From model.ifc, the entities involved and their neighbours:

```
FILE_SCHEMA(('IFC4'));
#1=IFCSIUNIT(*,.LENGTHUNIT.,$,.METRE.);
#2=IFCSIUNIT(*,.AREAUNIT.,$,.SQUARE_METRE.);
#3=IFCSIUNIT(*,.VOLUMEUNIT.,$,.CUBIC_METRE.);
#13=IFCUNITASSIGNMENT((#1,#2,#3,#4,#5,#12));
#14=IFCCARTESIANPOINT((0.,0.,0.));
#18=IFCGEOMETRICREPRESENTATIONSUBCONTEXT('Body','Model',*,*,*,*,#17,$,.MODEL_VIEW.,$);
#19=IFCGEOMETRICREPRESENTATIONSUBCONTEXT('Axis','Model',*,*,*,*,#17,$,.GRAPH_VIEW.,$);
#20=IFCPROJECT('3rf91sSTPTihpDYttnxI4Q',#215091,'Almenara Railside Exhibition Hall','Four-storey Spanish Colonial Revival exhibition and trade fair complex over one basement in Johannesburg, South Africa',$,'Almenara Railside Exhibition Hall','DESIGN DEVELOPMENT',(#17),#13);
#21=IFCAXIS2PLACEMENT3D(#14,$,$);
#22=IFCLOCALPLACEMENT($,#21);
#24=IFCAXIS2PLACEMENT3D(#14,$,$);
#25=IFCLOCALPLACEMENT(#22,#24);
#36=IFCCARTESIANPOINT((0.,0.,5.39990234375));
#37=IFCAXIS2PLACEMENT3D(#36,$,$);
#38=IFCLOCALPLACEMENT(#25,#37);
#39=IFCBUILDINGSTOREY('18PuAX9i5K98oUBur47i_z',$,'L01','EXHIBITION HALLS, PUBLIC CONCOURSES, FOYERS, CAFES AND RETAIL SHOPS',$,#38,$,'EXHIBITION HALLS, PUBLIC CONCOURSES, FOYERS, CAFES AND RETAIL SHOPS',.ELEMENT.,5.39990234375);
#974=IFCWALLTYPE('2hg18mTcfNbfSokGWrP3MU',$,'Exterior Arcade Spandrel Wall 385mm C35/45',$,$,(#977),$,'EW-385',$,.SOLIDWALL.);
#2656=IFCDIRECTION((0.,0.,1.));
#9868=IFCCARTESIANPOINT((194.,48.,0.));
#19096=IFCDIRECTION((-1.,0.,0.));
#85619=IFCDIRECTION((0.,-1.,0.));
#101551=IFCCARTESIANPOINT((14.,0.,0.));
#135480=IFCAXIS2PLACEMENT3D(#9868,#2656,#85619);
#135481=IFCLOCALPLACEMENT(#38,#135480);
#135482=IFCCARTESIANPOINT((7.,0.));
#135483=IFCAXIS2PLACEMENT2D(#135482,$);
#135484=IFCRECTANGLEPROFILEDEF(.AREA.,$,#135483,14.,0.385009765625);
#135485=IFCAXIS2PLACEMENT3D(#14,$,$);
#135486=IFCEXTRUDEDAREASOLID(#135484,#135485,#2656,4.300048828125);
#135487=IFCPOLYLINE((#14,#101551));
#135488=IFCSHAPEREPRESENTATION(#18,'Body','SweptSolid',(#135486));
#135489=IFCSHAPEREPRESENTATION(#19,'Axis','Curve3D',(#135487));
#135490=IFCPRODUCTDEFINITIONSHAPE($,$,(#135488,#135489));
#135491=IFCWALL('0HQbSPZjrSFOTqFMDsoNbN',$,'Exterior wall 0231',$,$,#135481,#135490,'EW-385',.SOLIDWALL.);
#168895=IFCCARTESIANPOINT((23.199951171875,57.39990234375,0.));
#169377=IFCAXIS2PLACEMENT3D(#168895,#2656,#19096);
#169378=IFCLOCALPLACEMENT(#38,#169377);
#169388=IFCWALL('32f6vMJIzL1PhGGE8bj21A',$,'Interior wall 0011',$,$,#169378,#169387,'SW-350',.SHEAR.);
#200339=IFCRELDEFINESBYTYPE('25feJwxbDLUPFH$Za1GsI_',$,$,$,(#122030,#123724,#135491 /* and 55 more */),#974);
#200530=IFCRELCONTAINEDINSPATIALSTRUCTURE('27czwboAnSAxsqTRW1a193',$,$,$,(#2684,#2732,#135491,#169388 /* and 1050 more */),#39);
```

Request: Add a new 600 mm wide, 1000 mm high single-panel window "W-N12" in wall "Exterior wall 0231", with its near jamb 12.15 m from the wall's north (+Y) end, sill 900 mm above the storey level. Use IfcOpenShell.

```python
import numpy as np
import ifcopenshell
import ifcopenshell.api.feature
import ifcopenshell.api.geometry
import ifcopenshell.api.root
import ifcopenshell.api.spatial
import ifcopenshell.geom
import ifcopenshell.util.element
import ifcopenshell.util.placement
import ifcopenshell.util.representation
import ifcopenshell.util.shape
import ifcopenshell.util.unit

model = ifcopenshell.open("model.ifc")
unit_scale = ifcopenshell.util.unit.calculate_unit_scale(model)
settings = ifcopenshell.geom.settings()


def volume(element):
    """Net volume in cubic metres, openings subtracted."""
    shape = ifcopenshell.geom.create_shape(settings, element)
    return ifcopenshell.util.shape.get_volume(shape.geometry)


wall = model.by_guid("0HQbSPZjrSFOTqFMDsoNbN")
storey = ifcopenshell.util.element.get_container(wall, ifc_class="IfcBuildingStorey")
context = ifcopenshell.util.representation.get_context(model, "Model", "Body", "MODEL_VIEW")
before = volume(wall)

width, height, from_end, sill = 0.6, 1, 12.15, 0.9  # metres

# The wall runs along its own X axis, and the end named is its -X end.
wall_shape = ifcopenshell.geom.create_shape(settings, wall)
x, y, z = ifcopenshell.util.shape.get_vertices(wall_shape.geometry).T
start = x.min() + from_end
face, thickness = float(y.min()), float(y.max() - y.min())
wall_matrix = ifcopenshell.util.placement.get_local_placement(wall.ObjectPlacement)
level = ifcopenshell.util.placement.get_local_placement(storey.ObjectPlacement)[2, 3]


def in_wall(x, y):
    """Placement at x, y metres in the wall's axes, at sill height."""
    matrix = wall_matrix.copy()
    matrix[:, 3] = wall_matrix @ np.array([x / unit_scale, y / unit_scale, 0.0, 1.0])
    matrix[2, 3] = level + sill / unit_scale
    return matrix


# Opening: a box that overshoots both wall faces by 50 mm.
opening = ifcopenshell.api.root.create_entity(model, ifc_class="IfcOpeningElement", predefined_type="OPENING")
box = ifcopenshell.api.geometry.add_wall_representation(
    model, context=context, length=width, height=height, thickness=thickness + 0.1
)
ifcopenshell.api.geometry.assign_representation(model, product=opening, representation=box)
ifcopenshell.api.geometry.edit_object_placement(model, product=opening, matrix=in_wall(start, face - 0.05), is_si=False)
ifcopenshell.api.feature.add_feature(model, feature=opening, element=wall)

window = ifcopenshell.api.root.create_entity(model, ifc_class="IfcWindow", name="W-N12", predefined_type="WINDOW")
window.OverallWidth, window.OverallHeight = width / unit_scale, height / unit_scale
window.PartitioningType = "SINGLE_PANEL"
body = ifcopenshell.api.geometry.add_window_representation(
    model,
    context=context,
    overall_width=window.OverallWidth,
    overall_height=window.OverallHeight,
    partition_type="SINGLE_PANEL",
)
ifcopenshell.api.geometry.assign_representation(model, product=window, representation=body)
ifcopenshell.api.spatial.assign_container(model, products=[window], relating_structure=storey)
ifcopenshell.api.feature.add_filling(model, opening=opening, element=window)

# Centre the window in the wall's thickness.
ifcopenshell.api.geometry.edit_object_placement(model, product=window, matrix=in_wall(start, face), is_si=False)
window_shape = ifcopenshell.geom.create_shape(settings, window)
depth = ifcopenshell.util.shape.get_vertices(window_shape.geometry)[:, 1]
offset = face + thickness / 2 - (depth.min() + depth.max()) / 2
ifcopenshell.api.geometry.edit_object_placement(model, product=window, matrix=in_wall(start, offset), is_si=False)

after = volume(wall)

print(f"wall volume {before:.3f} -> {after:.3f} m3")

model.write("model_rev.ifc")
```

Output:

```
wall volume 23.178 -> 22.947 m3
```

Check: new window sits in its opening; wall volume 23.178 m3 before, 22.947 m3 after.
